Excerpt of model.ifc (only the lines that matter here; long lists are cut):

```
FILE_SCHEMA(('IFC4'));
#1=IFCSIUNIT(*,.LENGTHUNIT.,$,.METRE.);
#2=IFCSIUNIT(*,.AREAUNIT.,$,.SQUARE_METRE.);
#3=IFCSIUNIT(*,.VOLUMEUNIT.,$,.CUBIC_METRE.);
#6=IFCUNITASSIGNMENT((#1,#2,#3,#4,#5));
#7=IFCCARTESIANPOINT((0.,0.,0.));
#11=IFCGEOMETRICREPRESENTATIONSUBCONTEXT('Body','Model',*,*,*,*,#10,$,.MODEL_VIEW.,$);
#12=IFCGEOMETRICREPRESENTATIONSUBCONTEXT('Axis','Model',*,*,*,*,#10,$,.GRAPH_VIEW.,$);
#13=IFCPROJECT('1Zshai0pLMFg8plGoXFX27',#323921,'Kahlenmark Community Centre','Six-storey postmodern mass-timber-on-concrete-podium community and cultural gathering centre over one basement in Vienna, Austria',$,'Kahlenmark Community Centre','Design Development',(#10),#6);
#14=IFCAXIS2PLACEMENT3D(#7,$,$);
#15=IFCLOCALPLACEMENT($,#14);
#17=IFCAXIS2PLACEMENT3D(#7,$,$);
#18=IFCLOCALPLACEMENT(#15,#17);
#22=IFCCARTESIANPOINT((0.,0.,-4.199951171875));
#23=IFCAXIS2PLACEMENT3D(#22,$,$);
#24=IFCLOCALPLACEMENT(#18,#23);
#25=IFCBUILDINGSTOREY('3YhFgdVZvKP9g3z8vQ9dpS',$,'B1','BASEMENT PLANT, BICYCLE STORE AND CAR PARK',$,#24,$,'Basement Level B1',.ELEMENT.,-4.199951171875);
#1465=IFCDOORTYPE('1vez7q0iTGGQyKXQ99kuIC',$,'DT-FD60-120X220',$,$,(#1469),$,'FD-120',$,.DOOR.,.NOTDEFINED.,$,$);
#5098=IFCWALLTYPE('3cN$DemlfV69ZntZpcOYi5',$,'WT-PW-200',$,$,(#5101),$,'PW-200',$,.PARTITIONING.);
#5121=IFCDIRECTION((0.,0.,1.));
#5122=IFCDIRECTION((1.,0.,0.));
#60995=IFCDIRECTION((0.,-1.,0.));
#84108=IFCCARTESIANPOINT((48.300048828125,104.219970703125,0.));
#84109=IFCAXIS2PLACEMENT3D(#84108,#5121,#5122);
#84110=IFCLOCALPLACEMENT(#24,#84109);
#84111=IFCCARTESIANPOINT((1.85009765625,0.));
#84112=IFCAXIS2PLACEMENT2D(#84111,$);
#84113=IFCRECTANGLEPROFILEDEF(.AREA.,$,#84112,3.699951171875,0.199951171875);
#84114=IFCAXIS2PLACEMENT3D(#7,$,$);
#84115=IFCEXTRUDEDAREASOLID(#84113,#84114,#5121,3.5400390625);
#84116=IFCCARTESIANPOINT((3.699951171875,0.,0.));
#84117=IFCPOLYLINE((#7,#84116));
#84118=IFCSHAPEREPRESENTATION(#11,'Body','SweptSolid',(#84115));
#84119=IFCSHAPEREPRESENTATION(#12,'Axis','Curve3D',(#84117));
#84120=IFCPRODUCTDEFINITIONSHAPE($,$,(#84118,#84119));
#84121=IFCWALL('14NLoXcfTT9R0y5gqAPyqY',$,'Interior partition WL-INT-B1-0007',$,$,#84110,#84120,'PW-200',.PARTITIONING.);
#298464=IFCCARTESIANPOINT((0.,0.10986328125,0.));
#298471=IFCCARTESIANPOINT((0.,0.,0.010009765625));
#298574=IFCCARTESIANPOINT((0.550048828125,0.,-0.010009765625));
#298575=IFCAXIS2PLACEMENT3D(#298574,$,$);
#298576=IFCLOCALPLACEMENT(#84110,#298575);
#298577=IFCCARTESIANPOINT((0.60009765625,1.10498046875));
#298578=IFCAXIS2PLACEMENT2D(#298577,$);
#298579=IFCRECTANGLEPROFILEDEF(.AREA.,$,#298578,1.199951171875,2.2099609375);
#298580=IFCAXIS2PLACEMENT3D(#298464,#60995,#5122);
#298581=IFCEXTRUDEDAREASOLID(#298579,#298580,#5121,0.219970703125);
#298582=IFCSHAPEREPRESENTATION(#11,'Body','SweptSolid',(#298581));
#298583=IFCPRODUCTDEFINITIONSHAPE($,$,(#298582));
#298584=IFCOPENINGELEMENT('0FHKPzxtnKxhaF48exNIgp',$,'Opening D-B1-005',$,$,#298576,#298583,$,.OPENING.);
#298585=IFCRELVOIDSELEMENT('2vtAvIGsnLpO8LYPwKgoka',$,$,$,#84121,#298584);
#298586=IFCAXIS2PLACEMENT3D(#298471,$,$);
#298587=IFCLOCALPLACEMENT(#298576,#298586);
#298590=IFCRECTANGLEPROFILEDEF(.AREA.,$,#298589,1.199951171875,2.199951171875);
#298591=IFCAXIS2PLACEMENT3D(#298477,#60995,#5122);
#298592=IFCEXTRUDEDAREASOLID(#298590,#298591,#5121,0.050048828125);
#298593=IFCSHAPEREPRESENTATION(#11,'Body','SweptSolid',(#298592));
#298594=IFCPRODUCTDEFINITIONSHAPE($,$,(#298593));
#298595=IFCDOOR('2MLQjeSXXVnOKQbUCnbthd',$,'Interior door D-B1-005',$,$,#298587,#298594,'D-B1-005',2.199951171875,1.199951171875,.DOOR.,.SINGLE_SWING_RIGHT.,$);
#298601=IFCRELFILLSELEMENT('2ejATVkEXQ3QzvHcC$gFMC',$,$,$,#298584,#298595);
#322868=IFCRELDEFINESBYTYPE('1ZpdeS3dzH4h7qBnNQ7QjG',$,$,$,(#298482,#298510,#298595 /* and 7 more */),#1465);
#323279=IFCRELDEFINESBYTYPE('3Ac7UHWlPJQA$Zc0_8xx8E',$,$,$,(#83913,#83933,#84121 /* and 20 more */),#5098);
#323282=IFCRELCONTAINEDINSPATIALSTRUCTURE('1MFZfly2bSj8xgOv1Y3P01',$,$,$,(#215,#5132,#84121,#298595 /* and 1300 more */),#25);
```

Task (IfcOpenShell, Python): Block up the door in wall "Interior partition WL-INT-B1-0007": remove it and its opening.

```python
import ifcopenshell
import ifcopenshell.api.feature
import ifcopenshell.api.root
import ifcopenshell.geom
import ifcopenshell.util.shape

model = ifcopenshell.open("model.ifc")
settings = ifcopenshell.geom.settings()


def volume(element):
    """Net volume in cubic metres, openings subtracted."""
    shape = ifcopenshell.geom.create_shape(settings, element)
    return ifcopenshell.util.shape.get_volume(shape.geometry)


door = model.by_guid("2MLQjeSXXVnOKQbUCnbthd")
opening = door.FillsVoids[0].RelatingOpeningElement
wall = opening.VoidsElements[0].RelatingBuildingElement
before = volume(wall)

ifcopenshell.api.root.remove_product(model, product=door)
ifcopenshell.api.feature.remove_feature(model, feature=opening)

after = volume(wall)

print(f"wall volume {before:.3f} -> {after:.3f} m3")

model.write("model_edited.ifc")
```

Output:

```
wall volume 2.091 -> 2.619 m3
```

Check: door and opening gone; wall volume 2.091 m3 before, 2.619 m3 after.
